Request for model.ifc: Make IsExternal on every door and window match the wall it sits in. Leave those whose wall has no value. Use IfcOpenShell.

First a look at what the model holds.

```python
import ifcopenshell
import ifcopenshell.util.element

model = ifcopenshell.open("model.ifc")
print(model.schema)
seen = {}
for e in model.by_type("IfcDoor") + model.by_type("IfcWindow"):
    if not e.FillsVoids:
        continue
    host = e.FillsVoids[0].RelatingOpeningElement.VoidsElements[0].RelatingBuildingElement
    own = ifcopenshell.util.element.get_pset(e, f"Pset_{e.is_a()[3:].removesuffix('StandardCase')}Common", "IsExternal")
    wall = ifcopenshell.util.element.get_pset(host, "Pset_WallCommon", "IsExternal")
    seen[e.is_a(), own, wall] = seen.get((e.is_a(), own, wall), 0) + 1
for (cls, own, wall), count in sorted(seen.items(), key=str):
    print(count, cls, "IsExternal:", own, "| host wall:", wall)
```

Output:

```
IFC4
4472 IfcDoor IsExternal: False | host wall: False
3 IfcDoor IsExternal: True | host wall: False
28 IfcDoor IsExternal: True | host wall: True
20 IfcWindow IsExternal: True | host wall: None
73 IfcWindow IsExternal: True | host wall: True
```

```python
import ifcopenshell
import ifcopenshell.api.pset
import ifcopenshell.util.element

model = ifcopenshell.open("model.ifc")

count = 0
for ifc_class, pset_name in (("IfcDoor", "Pset_DoorCommon"), ("IfcWindow", "Pset_WindowCommon")):
    for e in model.by_type(ifc_class):
        if not e.FillsVoids:
            continue
        host = e.FillsVoids[0].RelatingOpeningElement.VoidsElements[0].RelatingBuildingElement
        external = ifcopenshell.util.element.get_pset(host, "Pset_WallCommon", "IsExternal")
        if external is None or ifcopenshell.util.element.get_pset(e, pset_name, "IsExternal") == external:
            continue
        pset = ifcopenshell.api.pset.add_pset(model, product=e, name=pset_name)
        ifcopenshell.api.pset.edit_pset(model, pset=pset, properties={"IsExternal": external})
        count += 1

print(count, "updated")

model.write("model_v2.ifc")
```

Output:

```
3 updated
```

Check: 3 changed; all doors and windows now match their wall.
